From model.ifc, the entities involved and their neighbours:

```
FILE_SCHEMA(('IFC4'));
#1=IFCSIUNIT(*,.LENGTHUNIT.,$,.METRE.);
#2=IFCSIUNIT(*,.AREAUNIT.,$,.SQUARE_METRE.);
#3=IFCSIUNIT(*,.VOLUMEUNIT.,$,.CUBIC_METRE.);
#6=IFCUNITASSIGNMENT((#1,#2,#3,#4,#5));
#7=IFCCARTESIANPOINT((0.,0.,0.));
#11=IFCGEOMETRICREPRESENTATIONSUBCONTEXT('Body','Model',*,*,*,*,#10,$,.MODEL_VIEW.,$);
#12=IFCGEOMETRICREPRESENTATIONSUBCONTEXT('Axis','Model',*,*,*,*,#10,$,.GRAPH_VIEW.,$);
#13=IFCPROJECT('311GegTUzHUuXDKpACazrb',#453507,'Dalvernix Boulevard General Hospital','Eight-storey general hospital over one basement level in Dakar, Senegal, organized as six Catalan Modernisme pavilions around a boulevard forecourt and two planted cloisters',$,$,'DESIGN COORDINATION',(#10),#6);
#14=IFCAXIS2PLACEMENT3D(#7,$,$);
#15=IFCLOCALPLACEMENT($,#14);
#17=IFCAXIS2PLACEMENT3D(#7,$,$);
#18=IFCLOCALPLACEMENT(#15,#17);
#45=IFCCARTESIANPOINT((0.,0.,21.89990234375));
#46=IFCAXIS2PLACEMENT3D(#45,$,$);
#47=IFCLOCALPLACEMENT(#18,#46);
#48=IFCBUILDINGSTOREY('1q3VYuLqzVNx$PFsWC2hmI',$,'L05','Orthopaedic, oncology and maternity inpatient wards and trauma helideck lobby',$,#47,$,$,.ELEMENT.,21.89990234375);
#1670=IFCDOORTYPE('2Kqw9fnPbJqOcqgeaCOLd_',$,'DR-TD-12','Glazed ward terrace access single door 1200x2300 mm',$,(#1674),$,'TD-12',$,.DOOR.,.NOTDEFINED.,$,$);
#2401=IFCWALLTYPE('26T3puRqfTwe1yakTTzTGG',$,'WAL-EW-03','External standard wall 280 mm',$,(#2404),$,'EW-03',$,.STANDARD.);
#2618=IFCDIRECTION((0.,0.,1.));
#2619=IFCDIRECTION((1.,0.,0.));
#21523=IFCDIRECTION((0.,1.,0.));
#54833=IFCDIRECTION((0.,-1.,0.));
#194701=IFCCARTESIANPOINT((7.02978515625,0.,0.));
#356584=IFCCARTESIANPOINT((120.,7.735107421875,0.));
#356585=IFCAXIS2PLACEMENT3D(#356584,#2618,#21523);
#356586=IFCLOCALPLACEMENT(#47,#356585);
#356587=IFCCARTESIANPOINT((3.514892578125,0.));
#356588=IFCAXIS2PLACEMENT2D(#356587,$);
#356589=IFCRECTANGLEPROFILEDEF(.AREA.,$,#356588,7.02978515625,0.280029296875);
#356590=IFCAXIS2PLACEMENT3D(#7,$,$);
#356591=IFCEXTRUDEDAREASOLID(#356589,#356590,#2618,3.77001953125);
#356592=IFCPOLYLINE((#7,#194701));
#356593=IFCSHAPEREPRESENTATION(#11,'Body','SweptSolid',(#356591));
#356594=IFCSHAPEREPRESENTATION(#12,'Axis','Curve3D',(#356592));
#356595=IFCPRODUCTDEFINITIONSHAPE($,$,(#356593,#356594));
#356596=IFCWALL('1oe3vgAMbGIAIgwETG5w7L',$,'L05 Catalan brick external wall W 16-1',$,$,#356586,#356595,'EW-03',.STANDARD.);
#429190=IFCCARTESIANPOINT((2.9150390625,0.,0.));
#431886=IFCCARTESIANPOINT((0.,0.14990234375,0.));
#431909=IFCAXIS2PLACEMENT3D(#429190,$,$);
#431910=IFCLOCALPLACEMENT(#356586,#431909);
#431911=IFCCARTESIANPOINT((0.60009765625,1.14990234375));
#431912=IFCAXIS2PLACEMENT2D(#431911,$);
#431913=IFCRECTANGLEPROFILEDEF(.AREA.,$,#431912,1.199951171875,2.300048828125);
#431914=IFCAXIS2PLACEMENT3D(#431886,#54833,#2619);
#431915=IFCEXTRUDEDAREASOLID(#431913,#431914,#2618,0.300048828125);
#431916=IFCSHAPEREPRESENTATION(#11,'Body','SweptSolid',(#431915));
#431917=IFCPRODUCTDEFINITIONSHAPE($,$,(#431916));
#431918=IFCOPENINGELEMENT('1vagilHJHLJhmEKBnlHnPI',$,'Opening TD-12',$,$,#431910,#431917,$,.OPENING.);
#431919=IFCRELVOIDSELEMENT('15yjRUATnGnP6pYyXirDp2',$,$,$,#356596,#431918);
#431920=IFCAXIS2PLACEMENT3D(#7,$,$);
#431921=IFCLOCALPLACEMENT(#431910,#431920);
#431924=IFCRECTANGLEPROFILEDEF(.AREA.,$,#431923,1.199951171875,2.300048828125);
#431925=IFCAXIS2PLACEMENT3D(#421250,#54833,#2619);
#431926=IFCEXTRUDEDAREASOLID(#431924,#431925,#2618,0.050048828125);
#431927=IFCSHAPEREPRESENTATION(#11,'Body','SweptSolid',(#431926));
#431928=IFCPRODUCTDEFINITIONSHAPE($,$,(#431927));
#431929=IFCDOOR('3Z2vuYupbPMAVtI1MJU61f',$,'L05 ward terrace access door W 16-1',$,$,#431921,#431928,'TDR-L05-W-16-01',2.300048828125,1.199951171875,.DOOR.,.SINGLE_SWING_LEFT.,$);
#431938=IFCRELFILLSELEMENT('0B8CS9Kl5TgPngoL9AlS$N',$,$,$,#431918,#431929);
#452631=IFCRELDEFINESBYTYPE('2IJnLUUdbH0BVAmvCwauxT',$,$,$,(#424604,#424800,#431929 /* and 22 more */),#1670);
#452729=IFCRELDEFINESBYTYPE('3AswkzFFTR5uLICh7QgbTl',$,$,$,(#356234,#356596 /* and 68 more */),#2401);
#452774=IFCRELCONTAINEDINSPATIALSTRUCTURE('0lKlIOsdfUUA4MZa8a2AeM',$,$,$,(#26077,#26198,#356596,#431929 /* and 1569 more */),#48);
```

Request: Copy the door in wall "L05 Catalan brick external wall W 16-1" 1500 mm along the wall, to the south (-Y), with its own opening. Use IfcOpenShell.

```python
import ifcopenshell
import ifcopenshell.api.feature
import ifcopenshell.api.geometry
import ifcopenshell.api.root
import ifcopenshell.geom
import ifcopenshell.util.element
import ifcopenshell.util.placement
import ifcopenshell.util.shape

model = ifcopenshell.open("model.ifc")
settings = ifcopenshell.geom.settings()


def volume(element):
    """Net volume in cubic metres, openings subtracted."""
    shape = ifcopenshell.geom.create_shape(settings, element)
    return ifcopenshell.util.shape.get_volume(shape.geometry)


door = model.by_guid("3Z2vuYupbPMAVtI1MJU61f")
opening = door.FillsVoids[0].RelatingOpeningElement
wall = opening.VoidsElements[0].RelatingBuildingElement
before = volume(wall)
shift = ifcopenshell.util.placement.get_local_placement(wall.ObjectPlacement)[:3, 0] * -1.5

# copy_class copies the void relationship, type, container and properties, but no geometry.
new_opening = ifcopenshell.api.root.copy_class(model, product=opening)
new_opening.Representation = ifcopenshell.util.element.copy_deep(
    model, opening.Representation, exclude=["IfcGeometricRepresentationContext", "IfcRepresentationMap"]
)
new_door = ifcopenshell.api.root.copy_class(model, product=door)
new_door.Representation = ifcopenshell.util.element.copy_deep(
    model, door.Representation, exclude=["IfcGeometricRepresentationContext", "IfcRepresentationMap"]
)
new_door.Tag = None
ifcopenshell.api.feature.add_filling(model, opening=new_opening, element=new_door)

for old, new in ((opening, new_opening), (door, new_door)):
    matrix = ifcopenshell.util.placement.get_local_placement(old.ObjectPlacement)
    matrix[:3, 3] += shift
    ifcopenshell.api.geometry.edit_object_placement(model, product=new, matrix=matrix, is_si=False)

after = volume(wall)

print(f"wall volume {before:.3f} -> {after:.3f} m3")

model.write("model_rev.ifc")
```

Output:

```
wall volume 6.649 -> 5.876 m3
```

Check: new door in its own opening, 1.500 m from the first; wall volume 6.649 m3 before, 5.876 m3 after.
